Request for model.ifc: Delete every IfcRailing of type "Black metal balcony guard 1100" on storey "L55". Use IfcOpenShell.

First a look at what the model holds.

```python
import ifcopenshell
import ifcopenshell.util.element

model = ifcopenshell.open("model.ifc")
print(model.schema)
storey = next(s for s in model.by_type("IfcBuildingStorey") if s.Name == "L55")
railings = [e for e in ifcopenshell.util.element.get_decomposition(storey) if e.is_a("IfcRailing")]
seen = {}
for e in railings:
    element_type = ifcopenshell.util.element.get_type(e)
    name = element_type.Name if element_type not in (None, e) else None
    seen[name] = seen.get(name, 0) + 1
for name, count in sorted(seen.items(), key=str):
    print(count, "x", name)
```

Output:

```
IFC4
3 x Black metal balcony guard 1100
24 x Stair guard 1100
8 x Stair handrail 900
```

```python
import ifcopenshell
import ifcopenshell.api.root
import ifcopenshell.util.element

model = ifcopenshell.open("model.ifc")

storey = next(s for s in model.by_type("IfcBuildingStorey") if s.Name == "L55")
railings = [e for e in ifcopenshell.util.element.get_decomposition(storey) if e.is_a("IfcRailing")]
targets = [e for e in railings if (t := ifcopenshell.util.element.get_type(e)) not in (None, e) and t.Name == "Black metal balcony guard 1100"]

for e in targets:
    ifcopenshell.api.root.remove_product(model, product=e)
print(len(targets), "removed")

model.write("model_updated.ifc")
```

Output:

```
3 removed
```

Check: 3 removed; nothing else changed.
